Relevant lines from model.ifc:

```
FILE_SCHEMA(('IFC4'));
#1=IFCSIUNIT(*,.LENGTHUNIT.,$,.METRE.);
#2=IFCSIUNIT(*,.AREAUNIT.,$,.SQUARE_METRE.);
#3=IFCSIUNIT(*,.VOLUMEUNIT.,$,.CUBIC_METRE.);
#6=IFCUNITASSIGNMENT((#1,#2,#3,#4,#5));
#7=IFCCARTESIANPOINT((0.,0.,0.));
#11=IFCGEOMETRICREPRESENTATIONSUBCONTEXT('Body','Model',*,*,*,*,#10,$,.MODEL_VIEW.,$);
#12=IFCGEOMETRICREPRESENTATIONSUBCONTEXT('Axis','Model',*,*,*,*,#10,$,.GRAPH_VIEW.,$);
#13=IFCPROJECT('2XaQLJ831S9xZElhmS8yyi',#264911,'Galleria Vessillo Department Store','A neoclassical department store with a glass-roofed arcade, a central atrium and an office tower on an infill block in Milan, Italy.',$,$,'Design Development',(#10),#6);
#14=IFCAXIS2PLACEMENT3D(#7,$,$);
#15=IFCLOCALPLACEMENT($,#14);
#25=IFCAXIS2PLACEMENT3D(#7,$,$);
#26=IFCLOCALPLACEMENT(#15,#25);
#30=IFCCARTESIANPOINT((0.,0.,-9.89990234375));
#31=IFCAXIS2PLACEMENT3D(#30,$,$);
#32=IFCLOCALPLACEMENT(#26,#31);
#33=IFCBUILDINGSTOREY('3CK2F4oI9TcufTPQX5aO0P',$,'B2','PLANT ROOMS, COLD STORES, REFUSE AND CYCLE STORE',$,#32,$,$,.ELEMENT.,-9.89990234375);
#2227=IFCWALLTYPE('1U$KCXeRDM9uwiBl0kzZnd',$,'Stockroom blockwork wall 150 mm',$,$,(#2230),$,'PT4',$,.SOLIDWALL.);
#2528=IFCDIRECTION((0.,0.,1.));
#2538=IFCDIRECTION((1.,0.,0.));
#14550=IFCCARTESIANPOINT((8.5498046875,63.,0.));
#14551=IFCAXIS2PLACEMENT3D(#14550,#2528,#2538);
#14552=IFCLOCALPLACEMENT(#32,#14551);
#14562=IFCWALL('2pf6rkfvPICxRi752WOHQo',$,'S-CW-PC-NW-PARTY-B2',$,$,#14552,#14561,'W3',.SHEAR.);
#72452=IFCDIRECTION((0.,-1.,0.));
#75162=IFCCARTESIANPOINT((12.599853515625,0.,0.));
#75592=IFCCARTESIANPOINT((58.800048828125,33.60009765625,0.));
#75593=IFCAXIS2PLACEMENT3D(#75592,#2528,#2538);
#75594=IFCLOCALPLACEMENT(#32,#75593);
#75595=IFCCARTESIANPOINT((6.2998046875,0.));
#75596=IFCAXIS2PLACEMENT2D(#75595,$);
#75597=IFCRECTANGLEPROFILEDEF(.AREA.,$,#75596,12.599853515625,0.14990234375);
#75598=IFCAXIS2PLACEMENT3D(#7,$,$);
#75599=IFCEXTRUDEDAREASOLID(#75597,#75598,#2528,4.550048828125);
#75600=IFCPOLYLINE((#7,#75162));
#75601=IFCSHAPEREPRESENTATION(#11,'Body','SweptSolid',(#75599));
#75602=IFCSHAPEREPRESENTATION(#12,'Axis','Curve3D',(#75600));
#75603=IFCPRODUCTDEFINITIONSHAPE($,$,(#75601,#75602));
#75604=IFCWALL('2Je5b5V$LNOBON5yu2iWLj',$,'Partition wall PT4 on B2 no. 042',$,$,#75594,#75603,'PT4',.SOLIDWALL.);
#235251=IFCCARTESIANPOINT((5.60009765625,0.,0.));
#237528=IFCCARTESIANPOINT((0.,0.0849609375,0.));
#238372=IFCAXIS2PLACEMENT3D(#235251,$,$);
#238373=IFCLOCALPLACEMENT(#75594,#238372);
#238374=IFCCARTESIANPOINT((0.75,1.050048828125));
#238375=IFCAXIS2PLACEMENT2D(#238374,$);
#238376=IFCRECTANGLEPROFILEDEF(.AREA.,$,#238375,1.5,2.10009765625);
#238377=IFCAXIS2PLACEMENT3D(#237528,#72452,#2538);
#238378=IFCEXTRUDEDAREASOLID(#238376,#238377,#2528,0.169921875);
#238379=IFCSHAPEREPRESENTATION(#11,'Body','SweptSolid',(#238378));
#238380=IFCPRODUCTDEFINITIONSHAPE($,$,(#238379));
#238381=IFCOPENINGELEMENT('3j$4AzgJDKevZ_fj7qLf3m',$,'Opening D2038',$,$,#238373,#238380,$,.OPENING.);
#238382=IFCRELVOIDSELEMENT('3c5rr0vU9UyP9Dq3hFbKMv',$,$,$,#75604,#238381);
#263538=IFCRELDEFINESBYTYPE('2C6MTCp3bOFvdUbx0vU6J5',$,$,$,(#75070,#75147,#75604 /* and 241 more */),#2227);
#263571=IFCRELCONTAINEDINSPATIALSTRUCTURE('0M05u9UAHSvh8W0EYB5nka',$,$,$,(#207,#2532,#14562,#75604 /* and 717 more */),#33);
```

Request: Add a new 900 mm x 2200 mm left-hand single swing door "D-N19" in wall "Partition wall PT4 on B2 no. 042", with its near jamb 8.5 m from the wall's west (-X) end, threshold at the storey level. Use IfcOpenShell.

```python
import numpy as np
import ifcopenshell
import ifcopenshell.api.feature
import ifcopenshell.api.geometry
import ifcopenshell.api.root
import ifcopenshell.api.spatial
import ifcopenshell.geom
import ifcopenshell.util.element
import ifcopenshell.util.placement
import ifcopenshell.util.representation
import ifcopenshell.util.shape
import ifcopenshell.util.unit

model = ifcopenshell.open("model.ifc")
unit_scale = ifcopenshell.util.unit.calculate_unit_scale(model)
settings = ifcopenshell.geom.settings()


def volume(element):
    """Net volume in cubic metres, openings subtracted."""
    shape = ifcopenshell.geom.create_shape(settings, element)
    return ifcopenshell.util.shape.get_volume(shape.geometry)


wall = model.by_guid("2Je5b5V$LNOBON5yu2iWLj")
storey = ifcopenshell.util.element.get_container(wall, ifc_class="IfcBuildingStorey")
context = ifcopenshell.util.representation.get_context(model, "Model", "Body", "MODEL_VIEW")
before = volume(wall)

width, height, from_end, sill = 0.9, 2.2, 8.5, 0.0  # metres

# The wall runs along its own X axis, and the end named is its -X end.
wall_shape = ifcopenshell.geom.create_shape(settings, wall)
x, y, z = ifcopenshell.util.shape.get_vertices(wall_shape.geometry).T
start = x.min() + from_end
face, thickness = float(y.min()), float(y.max() - y.min())
wall_matrix = ifcopenshell.util.placement.get_local_placement(wall.ObjectPlacement)
level = ifcopenshell.util.placement.get_local_placement(storey.ObjectPlacement)[2, 3]


def in_wall(x, y):
    """Placement at x, y metres in the wall's axes, at sill height."""
    matrix = wall_matrix.copy()
    matrix[:, 3] = wall_matrix @ np.array([x / unit_scale, y / unit_scale, 0.0, 1.0])
    matrix[2, 3] = level + sill / unit_scale
    return matrix


# Opening: a box that overshoots both wall faces by 50 mm.
opening = ifcopenshell.api.root.create_entity(model, ifc_class="IfcOpeningElement", predefined_type="OPENING")
box = ifcopenshell.api.geometry.add_wall_representation(
    model, context=context, length=width, height=height, thickness=thickness + 0.1
)
ifcopenshell.api.geometry.assign_representation(model, product=opening, representation=box)
ifcopenshell.api.geometry.edit_object_placement(model, product=opening, matrix=in_wall(start, face - 0.05), is_si=False)
ifcopenshell.api.feature.add_feature(model, feature=opening, element=wall)

door = ifcopenshell.api.root.create_entity(model, ifc_class="IfcDoor", name="D-N19", predefined_type="DOOR")
door.OverallWidth, door.OverallHeight = width / unit_scale, height / unit_scale
door.OperationType = "SINGLE_SWING_LEFT"
body = ifcopenshell.api.geometry.add_door_representation(
    model,
    context=context,
    overall_width=door.OverallWidth,
    overall_height=door.OverallHeight,
    operation_type="SINGLE_SWING_LEFT",
    lining_properties={"LiningDepth": thickness / unit_scale, "ThresholdDepth": thickness / unit_scale},
)
ifcopenshell.api.geometry.assign_representation(model, product=door, representation=body)
ifcopenshell.api.spatial.assign_container(model, products=[door], relating_structure=storey)
ifcopenshell.api.feature.add_filling(model, opening=opening, element=door)

# The lining spans the wall, so the door starts at the wall face.
ifcopenshell.api.geometry.edit_object_placement(model, product=door, matrix=in_wall(start, face), is_si=False)

after = volume(wall)

print(f"wall volume {before:.3f} -> {after:.3f} m3")

model.write("model_edited.ifc")
```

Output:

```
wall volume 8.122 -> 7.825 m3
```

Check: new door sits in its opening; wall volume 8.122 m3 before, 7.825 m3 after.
